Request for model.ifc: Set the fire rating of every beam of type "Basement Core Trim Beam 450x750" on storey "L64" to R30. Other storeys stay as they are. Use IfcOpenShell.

First a look at what the model holds.

```python
import ifcopenshell
import ifcopenshell.util.element

model = ifcopenshell.open("model.ifc")
print(model.schema)
storey = next(s for s in model.by_type("IfcBuildingStorey") if s.Name == "L64")
beams = [e for e in ifcopenshell.util.element.get_decomposition(storey) if e.is_a("IfcBeam")]
seen = {}
for e in beams:
    element_type = ifcopenshell.util.element.get_type(e)
    key = (element_type.Name if element_type != e and element_type else None, ifcopenshell.util.element.get_pset(e, "Pset_BeamCommon", "FireRating"))
    seen[key] = seen.get(key, 0) + 1
for (name, value), count in sorted(seen.items(), key=str):
    print(count, "x", name, "|", value)
```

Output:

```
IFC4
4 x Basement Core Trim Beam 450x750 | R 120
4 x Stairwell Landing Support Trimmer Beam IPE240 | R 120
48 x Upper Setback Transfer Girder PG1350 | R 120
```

```python
import ifcopenshell
import ifcopenshell.api.pset
import ifcopenshell.util.element

model = ifcopenshell.open("model.ifc")

storey = next(s for s in model.by_type("IfcBuildingStorey") if s.Name == "L64")
beams = [e for e in ifcopenshell.util.element.get_decomposition(storey) if e.is_a("IfcBeam")]

count = 0
for e in beams:
    element_type = ifcopenshell.util.element.get_type(e)
    if element_type in (None, e) or element_type.Name != "Basement Core Trim Beam 450x750":
        continue
    found = ifcopenshell.util.element.get_pset(e, "Pset_BeamCommon", should_inherit=False)
    if found:
        pset = model.by_id(found["id"])
        if len(ifcopenshell.util.element.get_elements_by_pset(pset)) > 1:
            pset = ifcopenshell.api.pset.unshare_pset(model, products=[e], pset=pset)[0]
    else:
        pset = ifcopenshell.api.pset.add_pset(model, product=e, name="Pset_BeamCommon")
    ifcopenshell.api.pset.edit_pset(model, pset=pset, properties={"FireRating": "R30"})
    count += 1

print(count, "beams updated")

model.write("model_updated.ifc")
```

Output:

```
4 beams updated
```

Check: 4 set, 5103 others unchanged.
